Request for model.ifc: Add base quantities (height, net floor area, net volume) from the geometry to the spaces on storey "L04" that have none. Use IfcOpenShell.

First a look at what the model holds.

```python
import ifcopenshell
import ifcopenshell.util.element
import ifcopenshell.util.unit

model = ifcopenshell.open("model.ifc")
print(model.schema)
for unit_type in ("LENGTHUNIT", "AREAUNIT", "VOLUMEUNIT"):
    print(unit_type, ifcopenshell.util.unit.calculate_unit_scale(model, unit_type))
storey = next(s for s in model.by_type("IfcBuildingStorey") if s.Name == "L04")
spaces = [e for e in ifcopenshell.util.element.get_decomposition(storey) if e.is_a("IfcSpace")]
for e in sorted(spaces, key=lambda e: e.id()):
    print(e.id(), e.is_a(), e.Name, list(ifcopenshell.util.element.get_psets(e, qtos_only=True)), sep=" | ")
```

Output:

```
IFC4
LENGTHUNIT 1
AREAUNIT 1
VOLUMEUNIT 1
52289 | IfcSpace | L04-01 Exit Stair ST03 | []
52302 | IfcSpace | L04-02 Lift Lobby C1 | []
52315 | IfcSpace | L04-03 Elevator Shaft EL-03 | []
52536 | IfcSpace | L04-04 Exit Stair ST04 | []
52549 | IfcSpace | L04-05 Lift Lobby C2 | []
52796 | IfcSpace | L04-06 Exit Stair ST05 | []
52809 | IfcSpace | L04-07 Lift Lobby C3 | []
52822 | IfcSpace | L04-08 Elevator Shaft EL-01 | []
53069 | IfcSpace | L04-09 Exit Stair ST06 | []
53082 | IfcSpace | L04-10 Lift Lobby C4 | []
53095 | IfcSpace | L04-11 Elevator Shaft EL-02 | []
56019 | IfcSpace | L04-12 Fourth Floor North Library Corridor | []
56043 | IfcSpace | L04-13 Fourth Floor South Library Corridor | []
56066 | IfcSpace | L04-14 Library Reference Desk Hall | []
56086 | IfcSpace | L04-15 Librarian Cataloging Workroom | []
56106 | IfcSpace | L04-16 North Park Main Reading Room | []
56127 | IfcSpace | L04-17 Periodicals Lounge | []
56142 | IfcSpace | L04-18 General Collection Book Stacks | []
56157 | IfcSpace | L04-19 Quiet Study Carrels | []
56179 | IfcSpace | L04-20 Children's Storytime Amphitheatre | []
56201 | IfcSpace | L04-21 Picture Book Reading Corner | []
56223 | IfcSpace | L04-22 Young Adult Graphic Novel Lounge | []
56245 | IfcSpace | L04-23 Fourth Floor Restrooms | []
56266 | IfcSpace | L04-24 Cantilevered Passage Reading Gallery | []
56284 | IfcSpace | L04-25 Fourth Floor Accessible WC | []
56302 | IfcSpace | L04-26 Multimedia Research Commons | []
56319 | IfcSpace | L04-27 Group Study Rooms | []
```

```python
import ifcopenshell
import ifcopenshell.api.pset
import ifcopenshell.geom
import ifcopenshell.util.element
import ifcopenshell.util.shape
import ifcopenshell.util.unit

model = ifcopenshell.open("model.ifc")
unit_scale = ifcopenshell.util.unit.calculate_unit_scale(model)
area_scale = ifcopenshell.util.unit.calculate_unit_scale(model, "AREAUNIT")
volume_scale = ifcopenshell.util.unit.calculate_unit_scale(model, "VOLUMEUNIT")
settings = ifcopenshell.geom.settings()

storey = next(s for s in model.by_type("IfcBuildingStorey") if s.Name == "L04")
spaces = [e for e in ifcopenshell.util.element.get_decomposition(storey) if e.is_a("IfcSpace")]

for e in sorted(spaces, key=lambda e: e.id()):
    if ifcopenshell.util.element.get_psets(e, qtos_only=True, should_inherit=False):
        continue
    # Geometry comes back in metres, in the element's own axes.
    shape = ifcopenshell.geom.create_shape(settings, e)
    values = {
        "Height": ifcopenshell.util.shape.get_z(shape.geometry) / unit_scale,
        "NetFloorArea": ifcopenshell.util.shape.get_footprint_area(shape.geometry) / area_scale,
        "NetVolume": ifcopenshell.util.shape.get_volume(shape.geometry) / volume_scale,
    }
    qto = ifcopenshell.api.pset.add_qto(model, product=e, name="Qto_SpaceBaseQuantities")
    ifcopenshell.api.pset.edit_qto(model, qto=qto, properties=values)
    print(e.id(), {k: round(v, 3) for k, v in values.items()})

model.write("model_updated.ifc")
```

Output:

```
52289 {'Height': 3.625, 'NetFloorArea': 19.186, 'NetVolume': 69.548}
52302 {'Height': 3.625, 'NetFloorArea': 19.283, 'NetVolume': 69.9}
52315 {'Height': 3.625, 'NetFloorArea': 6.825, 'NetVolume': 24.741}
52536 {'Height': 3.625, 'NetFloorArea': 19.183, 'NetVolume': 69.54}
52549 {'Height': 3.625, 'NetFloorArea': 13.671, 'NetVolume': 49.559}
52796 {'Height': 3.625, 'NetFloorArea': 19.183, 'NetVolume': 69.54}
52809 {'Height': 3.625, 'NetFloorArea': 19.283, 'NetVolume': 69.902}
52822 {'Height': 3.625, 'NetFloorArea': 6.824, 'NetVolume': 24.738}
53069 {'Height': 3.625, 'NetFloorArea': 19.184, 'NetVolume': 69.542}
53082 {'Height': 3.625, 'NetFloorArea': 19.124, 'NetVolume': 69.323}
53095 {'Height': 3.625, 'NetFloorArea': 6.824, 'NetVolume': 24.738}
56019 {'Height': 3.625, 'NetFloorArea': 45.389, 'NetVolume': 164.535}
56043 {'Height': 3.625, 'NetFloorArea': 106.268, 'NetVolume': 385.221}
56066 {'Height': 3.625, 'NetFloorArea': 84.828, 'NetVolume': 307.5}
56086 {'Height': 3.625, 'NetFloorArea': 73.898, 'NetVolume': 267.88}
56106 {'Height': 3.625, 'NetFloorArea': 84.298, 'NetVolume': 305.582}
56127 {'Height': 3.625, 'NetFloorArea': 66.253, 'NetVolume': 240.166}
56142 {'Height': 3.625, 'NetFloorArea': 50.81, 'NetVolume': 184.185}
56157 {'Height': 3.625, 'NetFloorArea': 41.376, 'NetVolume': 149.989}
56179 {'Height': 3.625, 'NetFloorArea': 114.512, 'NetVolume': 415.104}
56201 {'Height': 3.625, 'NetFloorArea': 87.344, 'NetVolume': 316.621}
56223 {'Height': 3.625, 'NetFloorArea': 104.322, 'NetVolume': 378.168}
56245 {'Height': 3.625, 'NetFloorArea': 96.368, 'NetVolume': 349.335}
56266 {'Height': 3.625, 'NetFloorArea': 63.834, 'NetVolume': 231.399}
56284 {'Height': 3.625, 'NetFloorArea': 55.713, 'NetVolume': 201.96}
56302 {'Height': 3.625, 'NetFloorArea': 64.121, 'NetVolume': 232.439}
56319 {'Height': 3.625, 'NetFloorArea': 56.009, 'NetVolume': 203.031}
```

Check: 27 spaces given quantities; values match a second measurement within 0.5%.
